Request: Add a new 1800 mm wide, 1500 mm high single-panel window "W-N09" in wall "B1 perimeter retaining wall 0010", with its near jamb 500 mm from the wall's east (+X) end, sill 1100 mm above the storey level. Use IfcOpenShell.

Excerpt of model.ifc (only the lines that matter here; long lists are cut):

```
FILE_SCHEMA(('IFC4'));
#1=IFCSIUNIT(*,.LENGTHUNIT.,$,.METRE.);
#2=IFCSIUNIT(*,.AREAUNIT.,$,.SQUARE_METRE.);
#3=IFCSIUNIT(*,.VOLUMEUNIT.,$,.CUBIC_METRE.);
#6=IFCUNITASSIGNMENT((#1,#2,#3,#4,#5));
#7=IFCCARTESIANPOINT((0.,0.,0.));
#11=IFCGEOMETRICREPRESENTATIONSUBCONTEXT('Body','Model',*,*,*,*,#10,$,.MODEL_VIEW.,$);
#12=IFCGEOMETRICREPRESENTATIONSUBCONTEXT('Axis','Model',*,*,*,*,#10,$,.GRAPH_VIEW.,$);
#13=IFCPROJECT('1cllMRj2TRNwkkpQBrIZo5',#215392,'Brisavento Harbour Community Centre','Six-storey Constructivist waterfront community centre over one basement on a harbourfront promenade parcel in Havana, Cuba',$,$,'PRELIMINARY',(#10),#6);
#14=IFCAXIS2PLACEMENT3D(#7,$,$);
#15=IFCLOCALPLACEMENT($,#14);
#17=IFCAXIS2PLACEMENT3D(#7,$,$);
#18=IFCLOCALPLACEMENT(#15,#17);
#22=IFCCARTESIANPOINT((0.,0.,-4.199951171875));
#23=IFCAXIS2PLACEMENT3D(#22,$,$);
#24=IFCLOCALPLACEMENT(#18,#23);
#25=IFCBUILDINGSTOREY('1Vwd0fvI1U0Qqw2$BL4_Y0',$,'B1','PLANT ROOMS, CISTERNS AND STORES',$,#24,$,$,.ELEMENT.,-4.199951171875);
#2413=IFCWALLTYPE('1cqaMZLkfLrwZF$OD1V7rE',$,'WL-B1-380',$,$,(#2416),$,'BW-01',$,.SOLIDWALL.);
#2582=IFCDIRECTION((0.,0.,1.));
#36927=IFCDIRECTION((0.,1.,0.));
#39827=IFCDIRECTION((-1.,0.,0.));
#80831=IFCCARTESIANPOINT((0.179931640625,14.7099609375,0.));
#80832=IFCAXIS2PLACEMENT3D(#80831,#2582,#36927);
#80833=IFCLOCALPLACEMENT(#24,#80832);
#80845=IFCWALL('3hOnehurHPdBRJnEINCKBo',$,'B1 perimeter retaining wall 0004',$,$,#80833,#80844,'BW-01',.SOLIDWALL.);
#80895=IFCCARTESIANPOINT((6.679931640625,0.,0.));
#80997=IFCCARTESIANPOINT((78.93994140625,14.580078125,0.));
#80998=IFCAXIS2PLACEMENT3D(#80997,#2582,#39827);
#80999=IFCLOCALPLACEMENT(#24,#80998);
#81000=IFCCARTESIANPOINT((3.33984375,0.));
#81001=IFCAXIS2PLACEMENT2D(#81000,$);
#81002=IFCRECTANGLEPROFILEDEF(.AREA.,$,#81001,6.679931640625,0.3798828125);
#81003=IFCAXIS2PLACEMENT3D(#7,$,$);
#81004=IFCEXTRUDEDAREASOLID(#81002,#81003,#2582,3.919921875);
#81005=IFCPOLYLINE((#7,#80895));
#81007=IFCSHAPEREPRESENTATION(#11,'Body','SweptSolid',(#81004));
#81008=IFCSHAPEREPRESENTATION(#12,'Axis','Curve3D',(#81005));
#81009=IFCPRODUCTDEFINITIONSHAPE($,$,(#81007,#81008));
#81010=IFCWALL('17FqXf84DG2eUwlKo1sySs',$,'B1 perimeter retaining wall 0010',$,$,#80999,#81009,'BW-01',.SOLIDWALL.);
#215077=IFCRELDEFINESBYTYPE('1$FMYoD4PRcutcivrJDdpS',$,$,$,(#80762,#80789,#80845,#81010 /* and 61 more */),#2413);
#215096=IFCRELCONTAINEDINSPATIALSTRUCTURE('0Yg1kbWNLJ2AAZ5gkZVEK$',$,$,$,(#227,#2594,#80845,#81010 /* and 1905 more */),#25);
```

```python
import numpy as np
import ifcopenshell
import ifcopenshell.api.feature
import ifcopenshell.api.geometry
import ifcopenshell.api.root
import ifcopenshell.api.spatial
import ifcopenshell.geom
import ifcopenshell.util.element
import ifcopenshell.util.placement
import ifcopenshell.util.representation
import ifcopenshell.util.shape
import ifcopenshell.util.unit

model = ifcopenshell.open("model.ifc")
unit_scale = ifcopenshell.util.unit.calculate_unit_scale(model)
settings = ifcopenshell.geom.settings()


def volume(element):
    """Net volume in cubic metres, openings subtracted."""
    shape = ifcopenshell.geom.create_shape(settings, element)
    return ifcopenshell.util.shape.get_volume(shape.geometry)


wall = model.by_id(81010)
storey = ifcopenshell.util.element.get_container(wall, ifc_class="IfcBuildingStorey")
context = ifcopenshell.util.representation.get_context(model, "Model", "Body", "MODEL_VIEW")
before = volume(wall)

width, height, from_end, sill = 1.8, 1.5, 0.5, 1.1  # metres

# The wall runs along its own X axis, and the end named is its -X end.
wall_shape = ifcopenshell.geom.create_shape(settings, wall)
x, y, z = ifcopenshell.util.shape.get_vertices(wall_shape.geometry).T
start = x.min() + from_end
face, thickness = float(y.min()), float(y.max() - y.min())
wall_matrix = ifcopenshell.util.placement.get_local_placement(wall.ObjectPlacement)
level = ifcopenshell.util.placement.get_local_placement(storey.ObjectPlacement)[2, 3]


def in_wall(x, y):
    """Placement at x, y metres in the wall's axes, at sill height."""
    matrix = wall_matrix.copy()
    matrix[:, 3] = wall_matrix @ np.array([x / unit_scale, y / unit_scale, 0.0, 1.0])
    matrix[2, 3] = level + sill / unit_scale
    return matrix


# Opening: a box that overshoots both wall faces by 50 mm.
opening = ifcopenshell.api.root.create_entity(model, ifc_class="IfcOpeningElement", predefined_type="OPENING")
box = ifcopenshell.api.geometry.add_wall_representation(
    model, context=context, length=width, height=height, thickness=thickness + 0.1
)
ifcopenshell.api.geometry.assign_representation(model, product=opening, representation=box)
ifcopenshell.api.geometry.edit_object_placement(model, product=opening, matrix=in_wall(start, face - 0.05), is_si=False)
ifcopenshell.api.feature.add_feature(model, feature=opening, element=wall)

window = ifcopenshell.api.root.create_entity(model, ifc_class="IfcWindow", name="W-N09", predefined_type="WINDOW")
window.OverallWidth, window.OverallHeight = width / unit_scale, height / unit_scale
window.PartitioningType = "SINGLE_PANEL"
body = ifcopenshell.api.geometry.add_window_representation(
    model,
    context=context,
    overall_width=window.OverallWidth,
    overall_height=window.OverallHeight,
    partition_type="SINGLE_PANEL",
)
ifcopenshell.api.geometry.assign_representation(model, product=window, representation=body)
ifcopenshell.api.spatial.assign_container(model, products=[window], relating_structure=storey)
ifcopenshell.api.feature.add_filling(model, opening=opening, element=window)

# Centre the window in the wall's thickness.
ifcopenshell.api.geometry.edit_object_placement(model, product=window, matrix=in_wall(start, face), is_si=False)
window_shape = ifcopenshell.geom.create_shape(settings, window)
depth = ifcopenshell.util.shape.get_vertices(window_shape.geometry)[:, 1]
offset = face + thickness / 2 - (depth.min() + depth.max()) / 2
ifcopenshell.api.geometry.edit_object_placement(model, product=window, matrix=in_wall(start, offset), is_si=False)

after = volume(wall)

print(f"wall volume {before:.3f} -> {after:.3f} m3")

model.write("model_rev.ifc")
```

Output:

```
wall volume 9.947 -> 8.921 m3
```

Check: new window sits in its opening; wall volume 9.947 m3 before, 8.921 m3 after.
